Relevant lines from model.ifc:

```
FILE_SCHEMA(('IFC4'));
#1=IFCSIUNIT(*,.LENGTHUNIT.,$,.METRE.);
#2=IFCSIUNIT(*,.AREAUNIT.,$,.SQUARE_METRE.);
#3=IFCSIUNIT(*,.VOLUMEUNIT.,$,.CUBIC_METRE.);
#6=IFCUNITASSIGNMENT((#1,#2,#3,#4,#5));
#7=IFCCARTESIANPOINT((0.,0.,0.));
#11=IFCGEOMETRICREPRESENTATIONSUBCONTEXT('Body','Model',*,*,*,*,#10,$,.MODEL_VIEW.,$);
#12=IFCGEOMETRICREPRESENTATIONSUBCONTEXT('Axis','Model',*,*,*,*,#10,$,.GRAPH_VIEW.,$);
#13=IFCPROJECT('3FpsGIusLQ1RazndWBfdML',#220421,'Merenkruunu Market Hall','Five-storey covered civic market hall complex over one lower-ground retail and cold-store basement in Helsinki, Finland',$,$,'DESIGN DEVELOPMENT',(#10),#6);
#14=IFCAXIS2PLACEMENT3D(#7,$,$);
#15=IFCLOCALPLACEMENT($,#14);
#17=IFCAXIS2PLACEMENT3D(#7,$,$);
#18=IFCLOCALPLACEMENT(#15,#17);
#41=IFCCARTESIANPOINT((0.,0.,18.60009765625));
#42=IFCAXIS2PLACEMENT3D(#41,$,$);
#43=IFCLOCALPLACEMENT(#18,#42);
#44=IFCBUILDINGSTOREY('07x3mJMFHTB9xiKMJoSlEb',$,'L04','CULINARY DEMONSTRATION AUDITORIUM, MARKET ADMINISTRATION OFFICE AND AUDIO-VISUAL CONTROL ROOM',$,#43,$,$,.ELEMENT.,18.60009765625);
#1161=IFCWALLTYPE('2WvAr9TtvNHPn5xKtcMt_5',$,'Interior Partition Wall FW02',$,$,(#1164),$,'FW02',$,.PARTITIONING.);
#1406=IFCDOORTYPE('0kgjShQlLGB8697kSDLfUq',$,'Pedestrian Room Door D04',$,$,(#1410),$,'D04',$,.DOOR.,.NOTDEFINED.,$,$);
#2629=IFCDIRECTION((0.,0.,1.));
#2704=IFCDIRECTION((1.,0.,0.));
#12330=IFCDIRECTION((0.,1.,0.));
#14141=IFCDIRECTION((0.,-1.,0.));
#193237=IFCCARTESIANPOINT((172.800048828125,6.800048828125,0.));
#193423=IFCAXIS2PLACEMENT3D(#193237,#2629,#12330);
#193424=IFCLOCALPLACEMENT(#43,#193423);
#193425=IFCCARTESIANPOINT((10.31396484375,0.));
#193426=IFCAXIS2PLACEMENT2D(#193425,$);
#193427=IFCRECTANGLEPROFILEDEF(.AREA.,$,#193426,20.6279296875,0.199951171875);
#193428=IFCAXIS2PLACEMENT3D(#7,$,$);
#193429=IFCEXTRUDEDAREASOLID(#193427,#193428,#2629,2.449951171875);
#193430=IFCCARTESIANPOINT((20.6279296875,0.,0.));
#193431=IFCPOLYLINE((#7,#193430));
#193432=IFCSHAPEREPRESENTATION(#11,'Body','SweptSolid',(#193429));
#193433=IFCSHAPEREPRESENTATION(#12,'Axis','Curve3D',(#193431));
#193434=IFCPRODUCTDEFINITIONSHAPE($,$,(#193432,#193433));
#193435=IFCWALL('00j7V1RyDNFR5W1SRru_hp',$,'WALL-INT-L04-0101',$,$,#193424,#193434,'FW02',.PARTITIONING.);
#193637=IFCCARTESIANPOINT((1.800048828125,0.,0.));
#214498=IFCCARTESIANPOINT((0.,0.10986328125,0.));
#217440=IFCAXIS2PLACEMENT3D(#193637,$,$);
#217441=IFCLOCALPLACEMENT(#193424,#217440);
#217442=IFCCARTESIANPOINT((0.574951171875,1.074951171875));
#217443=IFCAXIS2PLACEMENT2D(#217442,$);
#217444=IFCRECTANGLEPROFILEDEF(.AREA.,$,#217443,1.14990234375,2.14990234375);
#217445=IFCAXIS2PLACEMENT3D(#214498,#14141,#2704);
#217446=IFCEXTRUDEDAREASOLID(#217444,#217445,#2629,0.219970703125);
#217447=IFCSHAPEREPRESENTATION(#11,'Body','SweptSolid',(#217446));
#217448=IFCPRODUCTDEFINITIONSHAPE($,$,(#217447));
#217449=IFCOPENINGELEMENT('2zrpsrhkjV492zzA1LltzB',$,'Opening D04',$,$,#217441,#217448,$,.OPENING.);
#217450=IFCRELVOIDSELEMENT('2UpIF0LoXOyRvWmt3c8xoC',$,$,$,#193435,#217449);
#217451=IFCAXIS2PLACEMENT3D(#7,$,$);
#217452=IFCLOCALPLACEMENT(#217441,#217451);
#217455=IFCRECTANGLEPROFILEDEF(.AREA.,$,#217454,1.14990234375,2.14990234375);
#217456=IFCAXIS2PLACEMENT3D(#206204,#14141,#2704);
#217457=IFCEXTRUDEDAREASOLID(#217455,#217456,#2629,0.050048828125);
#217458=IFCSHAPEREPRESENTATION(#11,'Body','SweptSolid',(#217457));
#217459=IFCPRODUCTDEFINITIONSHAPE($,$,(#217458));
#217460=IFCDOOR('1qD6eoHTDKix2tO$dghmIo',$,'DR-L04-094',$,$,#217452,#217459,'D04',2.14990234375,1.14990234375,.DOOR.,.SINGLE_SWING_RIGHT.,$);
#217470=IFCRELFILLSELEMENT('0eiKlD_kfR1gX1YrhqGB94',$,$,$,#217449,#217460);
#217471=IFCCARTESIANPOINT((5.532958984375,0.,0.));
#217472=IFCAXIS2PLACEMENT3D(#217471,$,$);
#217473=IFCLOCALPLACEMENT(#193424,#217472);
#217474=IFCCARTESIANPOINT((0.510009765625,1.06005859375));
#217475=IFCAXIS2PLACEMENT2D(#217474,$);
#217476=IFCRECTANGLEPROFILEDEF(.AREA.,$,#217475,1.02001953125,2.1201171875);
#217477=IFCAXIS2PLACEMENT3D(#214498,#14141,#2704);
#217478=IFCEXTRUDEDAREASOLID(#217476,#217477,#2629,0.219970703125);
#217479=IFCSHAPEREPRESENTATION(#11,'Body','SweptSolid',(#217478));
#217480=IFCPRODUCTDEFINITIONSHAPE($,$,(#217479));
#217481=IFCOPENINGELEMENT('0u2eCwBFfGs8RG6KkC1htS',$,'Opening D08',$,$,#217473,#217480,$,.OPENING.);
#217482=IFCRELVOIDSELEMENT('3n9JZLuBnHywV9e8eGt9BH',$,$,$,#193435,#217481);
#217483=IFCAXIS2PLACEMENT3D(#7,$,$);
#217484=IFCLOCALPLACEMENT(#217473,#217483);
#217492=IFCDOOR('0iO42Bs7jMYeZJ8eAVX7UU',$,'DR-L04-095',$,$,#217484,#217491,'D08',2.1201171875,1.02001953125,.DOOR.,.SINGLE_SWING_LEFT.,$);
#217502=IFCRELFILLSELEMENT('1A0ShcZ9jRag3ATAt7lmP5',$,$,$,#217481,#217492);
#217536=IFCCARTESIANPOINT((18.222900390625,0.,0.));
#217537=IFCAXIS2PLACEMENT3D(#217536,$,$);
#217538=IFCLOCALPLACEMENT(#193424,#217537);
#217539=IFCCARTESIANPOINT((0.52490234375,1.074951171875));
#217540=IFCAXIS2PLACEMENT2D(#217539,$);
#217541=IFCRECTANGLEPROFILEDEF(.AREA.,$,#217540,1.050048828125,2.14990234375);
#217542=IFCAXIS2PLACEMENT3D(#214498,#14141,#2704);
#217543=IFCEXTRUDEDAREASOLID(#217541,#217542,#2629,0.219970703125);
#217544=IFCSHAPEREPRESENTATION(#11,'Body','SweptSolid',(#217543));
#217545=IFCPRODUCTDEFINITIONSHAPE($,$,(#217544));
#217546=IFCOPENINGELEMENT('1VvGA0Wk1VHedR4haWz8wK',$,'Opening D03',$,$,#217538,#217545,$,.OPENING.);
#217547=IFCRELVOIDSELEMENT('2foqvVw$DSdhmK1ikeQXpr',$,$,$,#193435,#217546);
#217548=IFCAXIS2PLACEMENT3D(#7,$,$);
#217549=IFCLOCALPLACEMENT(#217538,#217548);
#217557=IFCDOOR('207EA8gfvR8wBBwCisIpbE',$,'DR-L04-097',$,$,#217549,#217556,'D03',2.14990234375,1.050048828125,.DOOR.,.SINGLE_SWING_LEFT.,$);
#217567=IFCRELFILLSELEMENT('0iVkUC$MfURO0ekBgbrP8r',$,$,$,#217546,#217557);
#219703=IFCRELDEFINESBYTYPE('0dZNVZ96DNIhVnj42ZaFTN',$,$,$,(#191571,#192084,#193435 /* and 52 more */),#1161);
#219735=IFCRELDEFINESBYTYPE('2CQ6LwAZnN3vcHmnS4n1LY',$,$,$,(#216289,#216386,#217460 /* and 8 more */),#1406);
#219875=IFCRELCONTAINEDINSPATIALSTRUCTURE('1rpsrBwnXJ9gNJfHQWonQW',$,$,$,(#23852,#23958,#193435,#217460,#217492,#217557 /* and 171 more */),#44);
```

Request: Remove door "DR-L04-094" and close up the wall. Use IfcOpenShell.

```python
import ifcopenshell
import ifcopenshell.api.feature
import ifcopenshell.api.root
import ifcopenshell.geom
import ifcopenshell.util.shape

model = ifcopenshell.open("model.ifc")
settings = ifcopenshell.geom.settings()


def volume(element):
    """Net volume in cubic metres, openings subtracted."""
    shape = ifcopenshell.geom.create_shape(settings, element)
    return ifcopenshell.util.shape.get_volume(shape.geometry)


door = model.by_guid("1qD6eoHTDKix2tO$dghmIo")
opening = door.FillsVoids[0].RelatingOpeningElement
wall = opening.VoidsElements[0].RelatingBuildingElement
before = volume(wall)

ifcopenshell.api.root.remove_product(model, product=door)
ifcopenshell.api.feature.remove_feature(model, feature=opening)

after = volume(wall)

print(f"wall volume {before:.3f} -> {after:.3f} m3")

model.write("model_updated.ifc")
```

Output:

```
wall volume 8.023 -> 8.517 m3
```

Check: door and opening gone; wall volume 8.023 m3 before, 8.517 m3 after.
